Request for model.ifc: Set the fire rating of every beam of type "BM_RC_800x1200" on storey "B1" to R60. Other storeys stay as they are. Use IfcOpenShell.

First a look at what the model holds.

```python
import ifcopenshell
import ifcopenshell.util.element

model = ifcopenshell.open("model.ifc")
print(model.schema)
storey = next(s for s in model.by_type("IfcBuildingStorey") if s.Name == "B1")
beams = [e for e in ifcopenshell.util.element.get_decomposition(storey) if e.is_a("IfcBeam")]
seen = {}
for e in beams:
    element_type = ifcopenshell.util.element.get_type(e)
    key = (element_type.Name if element_type != e and element_type else None, ifcopenshell.util.element.get_pset(e, "Pset_BeamCommon", "FireRating"))
    seen[key] = seen.get(key, 0) + 1
for (name, value), count in sorted(seen.items(), key=str):
    print(count, "x", name, "|", value)
```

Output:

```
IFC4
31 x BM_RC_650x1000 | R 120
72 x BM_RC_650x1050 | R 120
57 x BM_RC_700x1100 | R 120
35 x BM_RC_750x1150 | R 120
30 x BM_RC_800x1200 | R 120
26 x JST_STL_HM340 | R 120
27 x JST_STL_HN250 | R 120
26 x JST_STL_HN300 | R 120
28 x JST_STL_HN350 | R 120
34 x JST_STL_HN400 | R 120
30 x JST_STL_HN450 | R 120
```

```python
import ifcopenshell
import ifcopenshell.api.pset
import ifcopenshell.util.element

model = ifcopenshell.open("model.ifc")

storey = next(s for s in model.by_type("IfcBuildingStorey") if s.Name == "B1")
beams = [e for e in ifcopenshell.util.element.get_decomposition(storey) if e.is_a("IfcBeam")]

count = 0
for e in beams:
    element_type = ifcopenshell.util.element.get_type(e)
    if element_type in (None, e) or element_type.Name != "BM_RC_800x1200":
        continue
    # add_pset returns the element's existing set when there is one.
    pset = ifcopenshell.api.pset.add_pset(model, product=e, name="Pset_BeamCommon")
    ifcopenshell.api.pset.edit_pset(model, pset=pset, properties={"FireRating": "R60"})
    count += 1

print(count, "beams updated")

model.write("model_rev.ifc")
```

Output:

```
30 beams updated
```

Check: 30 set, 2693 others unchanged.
